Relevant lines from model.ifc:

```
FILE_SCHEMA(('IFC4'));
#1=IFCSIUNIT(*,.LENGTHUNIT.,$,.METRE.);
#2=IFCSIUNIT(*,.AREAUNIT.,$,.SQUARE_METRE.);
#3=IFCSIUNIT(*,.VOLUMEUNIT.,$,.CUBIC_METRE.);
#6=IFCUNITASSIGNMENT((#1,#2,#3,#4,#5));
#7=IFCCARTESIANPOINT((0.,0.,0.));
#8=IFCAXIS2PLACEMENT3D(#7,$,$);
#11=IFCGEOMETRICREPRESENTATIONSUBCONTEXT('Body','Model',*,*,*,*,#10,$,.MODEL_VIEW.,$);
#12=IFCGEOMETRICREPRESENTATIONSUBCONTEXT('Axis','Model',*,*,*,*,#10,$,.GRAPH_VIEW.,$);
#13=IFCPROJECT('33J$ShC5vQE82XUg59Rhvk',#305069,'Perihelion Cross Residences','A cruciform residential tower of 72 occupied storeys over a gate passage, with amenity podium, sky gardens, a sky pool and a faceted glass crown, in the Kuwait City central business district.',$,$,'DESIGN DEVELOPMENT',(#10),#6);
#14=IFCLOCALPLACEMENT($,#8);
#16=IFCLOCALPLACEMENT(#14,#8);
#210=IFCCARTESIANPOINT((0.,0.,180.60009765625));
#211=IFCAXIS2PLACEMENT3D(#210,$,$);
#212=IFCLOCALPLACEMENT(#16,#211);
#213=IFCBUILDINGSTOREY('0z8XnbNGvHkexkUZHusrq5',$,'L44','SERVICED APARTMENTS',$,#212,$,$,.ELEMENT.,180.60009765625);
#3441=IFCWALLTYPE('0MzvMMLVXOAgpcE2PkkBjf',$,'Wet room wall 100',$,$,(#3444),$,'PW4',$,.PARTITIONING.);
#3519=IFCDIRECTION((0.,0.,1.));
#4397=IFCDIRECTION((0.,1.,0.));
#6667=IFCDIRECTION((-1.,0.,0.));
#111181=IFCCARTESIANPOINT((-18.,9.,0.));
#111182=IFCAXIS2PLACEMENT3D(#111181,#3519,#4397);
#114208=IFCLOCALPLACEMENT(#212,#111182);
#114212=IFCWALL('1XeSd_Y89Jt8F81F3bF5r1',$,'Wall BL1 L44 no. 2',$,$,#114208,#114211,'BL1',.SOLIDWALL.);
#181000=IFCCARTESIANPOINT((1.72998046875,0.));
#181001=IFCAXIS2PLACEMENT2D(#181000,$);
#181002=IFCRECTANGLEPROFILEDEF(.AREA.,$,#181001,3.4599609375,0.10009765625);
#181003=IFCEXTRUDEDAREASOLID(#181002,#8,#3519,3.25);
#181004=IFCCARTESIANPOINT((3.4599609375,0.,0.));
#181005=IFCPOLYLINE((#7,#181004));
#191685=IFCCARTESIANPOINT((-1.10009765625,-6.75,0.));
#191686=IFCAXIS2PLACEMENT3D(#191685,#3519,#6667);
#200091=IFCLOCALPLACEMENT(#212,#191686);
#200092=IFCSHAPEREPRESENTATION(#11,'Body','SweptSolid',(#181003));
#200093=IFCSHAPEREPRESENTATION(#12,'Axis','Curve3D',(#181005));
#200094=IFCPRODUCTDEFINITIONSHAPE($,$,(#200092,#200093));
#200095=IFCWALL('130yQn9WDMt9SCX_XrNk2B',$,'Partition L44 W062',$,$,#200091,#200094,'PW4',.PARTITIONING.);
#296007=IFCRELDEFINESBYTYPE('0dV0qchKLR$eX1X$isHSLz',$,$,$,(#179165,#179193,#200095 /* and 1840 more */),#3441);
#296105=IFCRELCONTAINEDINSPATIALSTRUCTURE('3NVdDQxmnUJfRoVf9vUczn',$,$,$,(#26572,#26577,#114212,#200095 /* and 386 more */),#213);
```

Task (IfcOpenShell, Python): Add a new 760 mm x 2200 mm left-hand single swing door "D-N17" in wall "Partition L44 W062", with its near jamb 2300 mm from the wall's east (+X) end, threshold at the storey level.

```python
import numpy as np
import ifcopenshell
import ifcopenshell.api.feature
import ifcopenshell.api.geometry
import ifcopenshell.api.root
import ifcopenshell.api.spatial
import ifcopenshell.geom
import ifcopenshell.util.element
import ifcopenshell.util.placement
import ifcopenshell.util.representation
import ifcopenshell.util.shape
import ifcopenshell.util.unit

model = ifcopenshell.open("model.ifc")
unit_scale = ifcopenshell.util.unit.calculate_unit_scale(model)
settings = ifcopenshell.geom.settings()


def volume(element):
    """Net volume in cubic metres, openings subtracted."""
    shape = ifcopenshell.geom.create_shape(settings, element)
    return ifcopenshell.util.shape.get_volume(shape.geometry)


wall = model.by_id(200095)
storey = ifcopenshell.util.element.get_container(wall, ifc_class="IfcBuildingStorey")
context = ifcopenshell.util.representation.get_context(model, "Model", "Body", "MODEL_VIEW")
before = volume(wall)

width, height, from_end, sill = 0.76, 2.2, 2.3, 0.0  # metres

# The wall runs along its own X axis, and the end named is its -X end.
wall_shape = ifcopenshell.geom.create_shape(settings, wall)
x, y, z = ifcopenshell.util.shape.get_vertices(wall_shape.geometry).T
start = x.min() + from_end
face, thickness = float(y.min()), float(y.max() - y.min())
wall_matrix = ifcopenshell.util.placement.get_local_placement(wall.ObjectPlacement)
level = ifcopenshell.util.placement.get_local_placement(storey.ObjectPlacement)[2, 3]


def in_wall(x, y):
    """Placement at x, y metres in the wall's axes, at sill height."""
    matrix = wall_matrix.copy()
    matrix[:, 3] = wall_matrix @ np.array([x / unit_scale, y / unit_scale, 0.0, 1.0])
    matrix[2, 3] = level + sill / unit_scale
    return matrix


# Opening: a box that overshoots both wall faces by 50 mm.
opening = ifcopenshell.api.root.create_entity(model, ifc_class="IfcOpeningElement", predefined_type="OPENING")
box = ifcopenshell.api.geometry.add_wall_representation(
    model, context=context, length=width, height=height, thickness=thickness + 0.1
)
ifcopenshell.api.geometry.assign_representation(model, product=opening, representation=box)
ifcopenshell.api.geometry.edit_object_placement(model, product=opening, matrix=in_wall(start, face - 0.05), is_si=False)
ifcopenshell.api.feature.add_feature(model, feature=opening, element=wall)

door = ifcopenshell.api.root.create_entity(model, ifc_class="IfcDoor", name="D-N17", predefined_type="DOOR")
door.OverallWidth, door.OverallHeight = width / unit_scale, height / unit_scale
door.OperationType = "SINGLE_SWING_LEFT"
body = ifcopenshell.api.geometry.add_door_representation(
    model,
    context=context,
    overall_width=door.OverallWidth,
    overall_height=door.OverallHeight,
    operation_type="SINGLE_SWING_LEFT",
    lining_properties={"LiningDepth": thickness / unit_scale, "ThresholdDepth": thickness / unit_scale},
)
ifcopenshell.api.geometry.assign_representation(model, product=door, representation=body)
ifcopenshell.api.spatial.assign_container(model, products=[door], relating_structure=storey)
ifcopenshell.api.feature.add_filling(model, opening=opening, element=door)

# The lining spans the wall, so the door starts at the wall face.
ifcopenshell.api.geometry.edit_object_placement(model, product=door, matrix=in_wall(start, face), is_si=False)

after = volume(wall)

print(f"wall volume {before:.3f} -> {after:.3f} m3")

model.write("model_v2.ifc")
```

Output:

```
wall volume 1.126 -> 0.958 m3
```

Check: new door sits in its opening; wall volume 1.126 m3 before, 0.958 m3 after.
